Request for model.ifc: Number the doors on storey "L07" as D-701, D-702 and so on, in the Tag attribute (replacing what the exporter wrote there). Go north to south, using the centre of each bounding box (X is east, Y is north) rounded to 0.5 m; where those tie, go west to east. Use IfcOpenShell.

First a look at what the model holds.

```python
import ifcopenshell
import ifcopenshell.util.element
import ifcopenshell.util.placement

model = ifcopenshell.open("model.ifc")
print(model.schema)
storey = next(s for s in model.by_type("IfcBuildingStorey") if s.Name == "L07")
doors = [e for e in ifcopenshell.util.element.get_decomposition(storey) if e.is_a("IfcDoor")]
for e in sorted(doors, key=lambda e: e.id()):
    origin = ifcopenshell.util.placement.get_local_placement(e.ObjectPlacement)[:3, 3]
    print(e.id(), e.Tag, e.Name, origin.round(2) + 0.0, sep=" | ")
```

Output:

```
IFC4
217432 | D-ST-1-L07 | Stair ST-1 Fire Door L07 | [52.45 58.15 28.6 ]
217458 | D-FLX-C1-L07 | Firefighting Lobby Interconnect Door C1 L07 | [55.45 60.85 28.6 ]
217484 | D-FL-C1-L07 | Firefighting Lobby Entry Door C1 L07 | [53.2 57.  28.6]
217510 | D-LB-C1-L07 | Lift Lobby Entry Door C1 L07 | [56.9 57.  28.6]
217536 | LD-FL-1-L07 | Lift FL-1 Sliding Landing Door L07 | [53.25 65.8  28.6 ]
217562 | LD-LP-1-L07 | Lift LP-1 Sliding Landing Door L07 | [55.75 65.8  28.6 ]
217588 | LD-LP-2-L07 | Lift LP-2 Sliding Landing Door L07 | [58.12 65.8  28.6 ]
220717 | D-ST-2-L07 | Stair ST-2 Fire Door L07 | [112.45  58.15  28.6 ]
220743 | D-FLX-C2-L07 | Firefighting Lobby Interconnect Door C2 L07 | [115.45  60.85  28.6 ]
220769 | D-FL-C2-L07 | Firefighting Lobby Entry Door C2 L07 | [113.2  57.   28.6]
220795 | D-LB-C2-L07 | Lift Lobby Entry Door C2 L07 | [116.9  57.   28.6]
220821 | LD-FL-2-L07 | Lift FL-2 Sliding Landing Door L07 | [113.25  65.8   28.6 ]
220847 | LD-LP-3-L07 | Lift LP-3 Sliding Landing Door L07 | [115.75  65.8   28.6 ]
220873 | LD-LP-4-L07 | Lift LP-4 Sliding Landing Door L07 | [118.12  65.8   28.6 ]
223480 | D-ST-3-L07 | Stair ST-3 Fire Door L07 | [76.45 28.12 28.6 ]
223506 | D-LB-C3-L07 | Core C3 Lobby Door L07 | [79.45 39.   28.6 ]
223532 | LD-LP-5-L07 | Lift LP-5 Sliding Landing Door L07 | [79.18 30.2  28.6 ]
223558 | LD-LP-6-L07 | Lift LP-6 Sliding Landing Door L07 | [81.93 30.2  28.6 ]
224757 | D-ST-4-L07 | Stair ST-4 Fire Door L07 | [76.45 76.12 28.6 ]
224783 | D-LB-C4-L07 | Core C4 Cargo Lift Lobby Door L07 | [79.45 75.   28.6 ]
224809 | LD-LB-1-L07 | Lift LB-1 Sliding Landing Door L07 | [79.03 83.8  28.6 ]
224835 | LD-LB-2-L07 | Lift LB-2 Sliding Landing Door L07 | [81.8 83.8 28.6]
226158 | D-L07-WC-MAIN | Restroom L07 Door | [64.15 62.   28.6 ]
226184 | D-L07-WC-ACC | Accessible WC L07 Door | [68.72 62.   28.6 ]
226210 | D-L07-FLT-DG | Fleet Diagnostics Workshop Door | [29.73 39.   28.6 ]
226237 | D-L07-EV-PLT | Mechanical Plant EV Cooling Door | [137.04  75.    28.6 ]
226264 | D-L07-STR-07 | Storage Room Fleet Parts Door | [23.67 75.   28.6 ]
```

```python
import ifcopenshell
import ifcopenshell.geom
import ifcopenshell.util.element
import ifcopenshell.util.shape

model = ifcopenshell.open("model.ifc")
settings = ifcopenshell.geom.settings()
settings.set("use-world-coords", True)


def centre(element):
    shape = ifcopenshell.geom.create_shape(settings, element)
    return ifcopenshell.util.shape.get_bbox_centroid(shape.geometry)


storey = next(s for s in model.by_type("IfcBuildingStorey") if s.Name == "L07")
doors = [e for e in ifcopenshell.util.element.get_decomposition(storey) if e.is_a("IfcDoor")]

# Insertion points can sit at a corner or the storey origin, so sort by the geometry (in metres).
centres = {e: centre(e) for e in doors}
doors.sort(key=lambda e: (-round(centres[e][1] / 0.5), centres[e][0]))

for i, e in enumerate(doors, start=1):
    number = f"D-7{i:02d}"
    e.Tag = number
    print(e.id(), number)

model.write("model_updated.ifc")
```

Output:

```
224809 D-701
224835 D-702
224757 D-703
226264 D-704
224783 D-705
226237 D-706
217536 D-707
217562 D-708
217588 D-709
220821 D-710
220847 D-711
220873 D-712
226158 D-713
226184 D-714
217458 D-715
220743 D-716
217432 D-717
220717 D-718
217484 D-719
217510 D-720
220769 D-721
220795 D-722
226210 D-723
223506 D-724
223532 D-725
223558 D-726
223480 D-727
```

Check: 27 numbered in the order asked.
